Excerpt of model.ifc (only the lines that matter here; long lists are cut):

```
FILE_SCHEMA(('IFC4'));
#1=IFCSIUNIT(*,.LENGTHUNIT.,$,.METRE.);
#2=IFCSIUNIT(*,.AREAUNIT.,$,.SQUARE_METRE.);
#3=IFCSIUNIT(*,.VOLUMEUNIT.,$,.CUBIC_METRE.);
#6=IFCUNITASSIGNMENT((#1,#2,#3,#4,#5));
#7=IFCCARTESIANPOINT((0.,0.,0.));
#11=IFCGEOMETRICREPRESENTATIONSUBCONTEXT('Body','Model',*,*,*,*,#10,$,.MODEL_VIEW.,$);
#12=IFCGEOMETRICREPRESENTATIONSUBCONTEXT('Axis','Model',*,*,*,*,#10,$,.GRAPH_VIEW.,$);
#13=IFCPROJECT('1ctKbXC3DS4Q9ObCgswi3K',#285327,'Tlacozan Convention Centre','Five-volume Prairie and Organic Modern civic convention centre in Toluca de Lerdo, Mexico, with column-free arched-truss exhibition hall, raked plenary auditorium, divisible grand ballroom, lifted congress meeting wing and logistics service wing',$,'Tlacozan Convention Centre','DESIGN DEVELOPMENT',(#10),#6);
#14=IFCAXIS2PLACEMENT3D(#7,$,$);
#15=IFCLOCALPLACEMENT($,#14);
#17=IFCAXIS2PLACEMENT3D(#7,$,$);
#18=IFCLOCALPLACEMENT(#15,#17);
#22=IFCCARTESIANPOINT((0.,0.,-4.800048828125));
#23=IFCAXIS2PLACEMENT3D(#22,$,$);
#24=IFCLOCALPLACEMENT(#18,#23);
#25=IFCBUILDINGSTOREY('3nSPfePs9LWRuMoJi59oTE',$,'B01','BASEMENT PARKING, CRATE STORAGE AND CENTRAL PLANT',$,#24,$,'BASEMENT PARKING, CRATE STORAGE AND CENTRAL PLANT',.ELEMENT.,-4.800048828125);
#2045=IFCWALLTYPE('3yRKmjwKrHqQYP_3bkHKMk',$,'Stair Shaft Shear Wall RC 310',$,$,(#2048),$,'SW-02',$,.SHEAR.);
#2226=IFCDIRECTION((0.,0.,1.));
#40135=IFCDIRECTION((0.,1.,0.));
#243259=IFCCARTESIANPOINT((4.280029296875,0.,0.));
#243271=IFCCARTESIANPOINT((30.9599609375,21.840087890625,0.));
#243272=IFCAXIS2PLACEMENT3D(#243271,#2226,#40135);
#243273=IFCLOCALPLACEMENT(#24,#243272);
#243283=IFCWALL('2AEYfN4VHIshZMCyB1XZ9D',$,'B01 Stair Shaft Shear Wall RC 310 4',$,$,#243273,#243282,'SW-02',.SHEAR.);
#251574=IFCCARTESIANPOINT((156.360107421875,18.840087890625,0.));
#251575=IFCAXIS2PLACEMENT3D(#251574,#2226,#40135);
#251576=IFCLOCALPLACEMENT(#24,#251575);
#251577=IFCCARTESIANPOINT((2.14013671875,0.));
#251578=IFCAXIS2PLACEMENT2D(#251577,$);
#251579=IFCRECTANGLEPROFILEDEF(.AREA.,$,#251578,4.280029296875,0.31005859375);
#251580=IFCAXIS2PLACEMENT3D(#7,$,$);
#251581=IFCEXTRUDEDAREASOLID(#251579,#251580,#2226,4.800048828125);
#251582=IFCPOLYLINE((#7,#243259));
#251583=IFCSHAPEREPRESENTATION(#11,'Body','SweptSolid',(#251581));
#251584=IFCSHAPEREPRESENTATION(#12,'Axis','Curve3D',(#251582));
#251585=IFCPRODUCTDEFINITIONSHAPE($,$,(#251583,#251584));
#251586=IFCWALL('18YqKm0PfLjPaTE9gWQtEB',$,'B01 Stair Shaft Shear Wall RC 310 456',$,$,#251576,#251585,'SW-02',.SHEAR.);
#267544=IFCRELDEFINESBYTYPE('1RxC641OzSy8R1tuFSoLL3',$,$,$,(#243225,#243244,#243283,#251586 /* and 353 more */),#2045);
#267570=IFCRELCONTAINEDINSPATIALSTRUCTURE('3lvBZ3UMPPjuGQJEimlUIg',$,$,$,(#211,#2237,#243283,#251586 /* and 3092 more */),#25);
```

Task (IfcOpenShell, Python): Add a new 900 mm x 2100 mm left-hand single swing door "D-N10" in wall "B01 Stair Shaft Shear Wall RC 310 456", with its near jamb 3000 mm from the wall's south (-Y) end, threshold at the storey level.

```python
import numpy as np
import ifcopenshell
import ifcopenshell.api.feature
import ifcopenshell.api.geometry
import ifcopenshell.api.root
import ifcopenshell.api.spatial
import ifcopenshell.geom
import ifcopenshell.util.element
import ifcopenshell.util.placement
import ifcopenshell.util.representation
import ifcopenshell.util.shape
import ifcopenshell.util.unit

model = ifcopenshell.open("model.ifc")
unit_scale = ifcopenshell.util.unit.calculate_unit_scale(model)
settings = ifcopenshell.geom.settings()


def volume(element):
    """Net volume in cubic metres, openings subtracted."""
    shape = ifcopenshell.geom.create_shape(settings, element)
    return ifcopenshell.util.shape.get_volume(shape.geometry)


wall = model.by_guid("18YqKm0PfLjPaTE9gWQtEB")
storey = ifcopenshell.util.element.get_container(wall, ifc_class="IfcBuildingStorey")
context = ifcopenshell.util.representation.get_context(model, "Model", "Body", "MODEL_VIEW")
before = volume(wall)

width, height, from_end, sill = 0.9, 2.1, 3, 0.0  # metres

# The wall runs along its own X axis, and the end named is its -X end.
wall_shape = ifcopenshell.geom.create_shape(settings, wall)
x, y, z = ifcopenshell.util.shape.get_vertices(wall_shape.geometry).T
start = x.min() + from_end
face, thickness = float(y.min()), float(y.max() - y.min())
wall_matrix = ifcopenshell.util.placement.get_local_placement(wall.ObjectPlacement)
level = ifcopenshell.util.placement.get_local_placement(storey.ObjectPlacement)[2, 3]


def in_wall(x, y):
    """Placement at x, y metres in the wall's axes, at sill height."""
    matrix = wall_matrix.copy()
    matrix[:, 3] = wall_matrix @ np.array([x / unit_scale, y / unit_scale, 0.0, 1.0])
    matrix[2, 3] = level + sill / unit_scale
    return matrix


# Opening: a box that overshoots both wall faces by 50 mm.
opening = ifcopenshell.api.root.create_entity(model, ifc_class="IfcOpeningElement", predefined_type="OPENING")
box = ifcopenshell.api.geometry.add_wall_representation(
    model, context=context, length=width, height=height, thickness=thickness + 0.1
)
ifcopenshell.api.geometry.assign_representation(model, product=opening, representation=box)
ifcopenshell.api.geometry.edit_object_placement(model, product=opening, matrix=in_wall(start, face - 0.05), is_si=False)
ifcopenshell.api.feature.add_feature(model, feature=opening, element=wall)

door = ifcopenshell.api.root.create_entity(model, ifc_class="IfcDoor", name="D-N10", predefined_type="DOOR")
door.OverallWidth, door.OverallHeight = width / unit_scale, height / unit_scale
door.OperationType = "SINGLE_SWING_LEFT"
body = ifcopenshell.api.geometry.add_door_representation(
    model,
    context=context,
    overall_width=door.OverallWidth,
    overall_height=door.OverallHeight,
    operation_type="SINGLE_SWING_LEFT",
    lining_properties={"LiningDepth": thickness / unit_scale, "ThresholdDepth": thickness / unit_scale},
)
ifcopenshell.api.geometry.assign_representation(model, product=door, representation=body)
ifcopenshell.api.spatial.assign_container(model, products=[door], relating_structure=storey)
ifcopenshell.api.feature.add_filling(model, opening=opening, element=door)

# The lining spans the wall, so the door starts at the wall face.
ifcopenshell.api.geometry.edit_object_placement(model, product=door, matrix=in_wall(start, face), is_si=False)

after = volume(wall)

print(f"wall volume {before:.3f} -> {after:.3f} m3")

model.write("model-out.ifc")
```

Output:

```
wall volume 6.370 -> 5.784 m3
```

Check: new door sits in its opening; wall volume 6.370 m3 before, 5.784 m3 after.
